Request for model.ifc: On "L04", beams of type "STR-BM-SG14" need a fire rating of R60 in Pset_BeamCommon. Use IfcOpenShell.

First a look at what the model holds.

```python
import ifcopenshell
import ifcopenshell.util.element

model = ifcopenshell.open("model.ifc")
print(model.schema)
storey = next(s for s in model.by_type("IfcBuildingStorey") if s.Name == "L04")
beams = [e for e in ifcopenshell.util.element.get_decomposition(storey) if e.is_a("IfcBeam")]
seen = {}
for e in beams:
    element_type = ifcopenshell.util.element.get_type(e)
    key = (element_type.Name if element_type != e and element_type else None, ifcopenshell.util.element.get_pset(e, "Pset_BeamCommon", "FireRating"))
    seen[key] = seen.get(key, 0) + 1
for (name, value), count in sorted(seen.items(), key=str):
    print(count, "x", name, "|", value)
```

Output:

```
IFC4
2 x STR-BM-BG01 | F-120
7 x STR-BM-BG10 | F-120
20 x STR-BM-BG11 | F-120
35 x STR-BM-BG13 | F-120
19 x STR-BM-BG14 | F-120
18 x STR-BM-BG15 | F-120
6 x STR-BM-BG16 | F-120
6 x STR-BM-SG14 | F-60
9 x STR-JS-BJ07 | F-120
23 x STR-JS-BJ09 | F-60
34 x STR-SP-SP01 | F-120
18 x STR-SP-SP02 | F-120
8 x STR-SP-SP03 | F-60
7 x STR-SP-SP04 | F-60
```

```python
import ifcopenshell
import ifcopenshell.api.pset
import ifcopenshell.util.element

model = ifcopenshell.open("model.ifc")

storey = next(s for s in model.by_type("IfcBuildingStorey") if s.Name == "L04")
beams = [e for e in ifcopenshell.util.element.get_decomposition(storey) if e.is_a("IfcBeam")]

count = 0
for e in beams:
    element_type = ifcopenshell.util.element.get_type(e)
    if element_type in (None, e) or element_type.Name != "STR-BM-SG14":
        continue
    # add_pset returns the element's existing set when there is one.
    pset = ifcopenshell.api.pset.add_pset(model, product=e, name="Pset_BeamCommon")
    ifcopenshell.api.pset.edit_pset(model, pset=pset, properties={"FireRating": "R60"})
    count += 1

print(count, "beams updated")

model.write("model_updated.ifc")
```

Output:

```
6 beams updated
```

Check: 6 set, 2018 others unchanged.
